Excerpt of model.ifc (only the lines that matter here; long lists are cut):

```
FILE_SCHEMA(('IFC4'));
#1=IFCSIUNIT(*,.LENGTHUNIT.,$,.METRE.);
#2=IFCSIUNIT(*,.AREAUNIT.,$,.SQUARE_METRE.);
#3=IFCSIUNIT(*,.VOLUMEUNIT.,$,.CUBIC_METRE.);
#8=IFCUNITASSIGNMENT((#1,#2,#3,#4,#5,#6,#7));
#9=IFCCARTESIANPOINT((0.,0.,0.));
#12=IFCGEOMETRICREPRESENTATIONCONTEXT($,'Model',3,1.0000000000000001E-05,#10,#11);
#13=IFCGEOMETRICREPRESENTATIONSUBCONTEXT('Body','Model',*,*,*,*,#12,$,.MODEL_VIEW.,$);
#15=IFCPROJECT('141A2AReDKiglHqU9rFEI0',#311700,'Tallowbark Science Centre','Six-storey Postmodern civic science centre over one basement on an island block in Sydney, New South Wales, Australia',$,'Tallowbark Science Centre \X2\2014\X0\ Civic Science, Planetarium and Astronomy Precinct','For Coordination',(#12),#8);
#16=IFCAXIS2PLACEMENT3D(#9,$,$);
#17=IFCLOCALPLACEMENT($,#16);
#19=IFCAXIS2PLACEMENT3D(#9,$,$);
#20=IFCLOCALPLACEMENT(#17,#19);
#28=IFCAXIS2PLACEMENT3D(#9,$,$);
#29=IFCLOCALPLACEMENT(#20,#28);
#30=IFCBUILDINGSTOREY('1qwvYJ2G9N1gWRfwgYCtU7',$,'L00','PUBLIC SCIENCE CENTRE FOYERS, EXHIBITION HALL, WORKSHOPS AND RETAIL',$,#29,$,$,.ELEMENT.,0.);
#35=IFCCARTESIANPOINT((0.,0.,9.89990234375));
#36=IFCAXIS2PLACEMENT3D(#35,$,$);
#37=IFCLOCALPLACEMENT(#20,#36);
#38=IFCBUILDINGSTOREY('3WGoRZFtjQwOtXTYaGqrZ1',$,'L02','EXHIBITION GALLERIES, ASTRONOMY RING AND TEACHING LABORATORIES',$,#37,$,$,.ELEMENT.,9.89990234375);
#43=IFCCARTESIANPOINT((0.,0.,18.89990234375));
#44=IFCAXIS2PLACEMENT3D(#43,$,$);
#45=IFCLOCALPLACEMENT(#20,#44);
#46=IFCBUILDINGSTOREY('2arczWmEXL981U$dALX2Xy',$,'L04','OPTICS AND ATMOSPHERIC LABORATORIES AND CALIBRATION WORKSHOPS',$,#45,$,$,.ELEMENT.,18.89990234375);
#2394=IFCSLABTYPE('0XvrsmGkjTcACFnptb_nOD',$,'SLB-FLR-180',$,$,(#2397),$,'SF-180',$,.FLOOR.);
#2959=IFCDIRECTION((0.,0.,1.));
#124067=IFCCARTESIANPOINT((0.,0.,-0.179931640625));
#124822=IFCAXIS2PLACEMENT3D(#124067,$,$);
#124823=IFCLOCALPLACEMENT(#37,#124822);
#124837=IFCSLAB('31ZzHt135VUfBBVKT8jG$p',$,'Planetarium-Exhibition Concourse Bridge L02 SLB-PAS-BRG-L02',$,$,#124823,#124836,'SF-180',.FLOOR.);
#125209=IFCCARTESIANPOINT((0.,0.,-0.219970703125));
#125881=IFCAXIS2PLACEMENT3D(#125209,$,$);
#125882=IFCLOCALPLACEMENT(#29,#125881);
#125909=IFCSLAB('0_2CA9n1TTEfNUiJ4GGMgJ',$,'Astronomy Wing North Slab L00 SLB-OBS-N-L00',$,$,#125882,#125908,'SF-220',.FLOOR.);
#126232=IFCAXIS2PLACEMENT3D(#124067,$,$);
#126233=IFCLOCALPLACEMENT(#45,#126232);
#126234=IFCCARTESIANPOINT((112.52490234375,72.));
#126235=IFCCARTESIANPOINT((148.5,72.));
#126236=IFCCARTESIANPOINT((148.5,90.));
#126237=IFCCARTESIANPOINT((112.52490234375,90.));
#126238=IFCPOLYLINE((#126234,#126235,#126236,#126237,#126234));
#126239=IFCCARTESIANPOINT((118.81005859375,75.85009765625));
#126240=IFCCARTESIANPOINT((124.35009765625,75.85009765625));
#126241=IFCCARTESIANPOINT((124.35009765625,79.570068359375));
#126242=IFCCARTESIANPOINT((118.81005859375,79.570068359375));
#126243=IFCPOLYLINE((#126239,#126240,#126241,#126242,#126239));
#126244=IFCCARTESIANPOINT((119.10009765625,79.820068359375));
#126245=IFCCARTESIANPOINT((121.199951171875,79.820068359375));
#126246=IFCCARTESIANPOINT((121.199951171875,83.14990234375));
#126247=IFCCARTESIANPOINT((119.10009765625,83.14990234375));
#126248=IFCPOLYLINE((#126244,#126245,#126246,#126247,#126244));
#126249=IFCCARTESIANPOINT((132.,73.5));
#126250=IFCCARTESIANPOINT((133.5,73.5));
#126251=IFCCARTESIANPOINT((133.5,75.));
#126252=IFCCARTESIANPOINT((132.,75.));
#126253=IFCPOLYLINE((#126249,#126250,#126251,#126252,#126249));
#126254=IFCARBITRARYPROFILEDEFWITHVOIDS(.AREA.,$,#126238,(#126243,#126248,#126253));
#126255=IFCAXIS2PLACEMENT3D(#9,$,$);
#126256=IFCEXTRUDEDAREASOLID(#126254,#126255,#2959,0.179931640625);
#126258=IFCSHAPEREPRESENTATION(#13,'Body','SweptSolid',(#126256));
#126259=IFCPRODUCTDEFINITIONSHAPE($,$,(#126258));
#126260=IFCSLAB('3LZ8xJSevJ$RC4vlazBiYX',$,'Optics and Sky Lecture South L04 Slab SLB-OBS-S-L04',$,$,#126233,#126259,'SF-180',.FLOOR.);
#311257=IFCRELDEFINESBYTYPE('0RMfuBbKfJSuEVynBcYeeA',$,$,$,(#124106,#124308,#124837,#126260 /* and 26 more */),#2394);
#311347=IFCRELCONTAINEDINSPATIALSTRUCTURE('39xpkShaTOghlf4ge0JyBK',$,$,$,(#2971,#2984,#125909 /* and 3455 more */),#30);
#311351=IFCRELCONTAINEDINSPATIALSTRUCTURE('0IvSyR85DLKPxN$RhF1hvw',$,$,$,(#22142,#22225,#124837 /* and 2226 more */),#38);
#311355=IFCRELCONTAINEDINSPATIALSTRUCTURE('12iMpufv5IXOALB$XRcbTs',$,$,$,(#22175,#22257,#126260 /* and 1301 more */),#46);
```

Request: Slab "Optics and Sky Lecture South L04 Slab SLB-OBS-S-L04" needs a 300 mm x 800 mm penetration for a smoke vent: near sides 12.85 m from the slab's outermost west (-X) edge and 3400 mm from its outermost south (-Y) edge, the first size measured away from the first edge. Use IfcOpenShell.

```python
import numpy as np
import ifcopenshell
import ifcopenshell.api.feature
import ifcopenshell.api.geometry
import ifcopenshell.api.root
import ifcopenshell.geom
import ifcopenshell.util.placement
import ifcopenshell.util.representation
import ifcopenshell.util.shape
import ifcopenshell.util.unit

model = ifcopenshell.open("model.ifc")
unit_scale = ifcopenshell.util.unit.calculate_unit_scale(model)
settings = ifcopenshell.geom.settings()


def volume(element):
    """Net volume in cubic metres, openings subtracted."""
    shape = ifcopenshell.geom.create_shape(settings, element)
    return ifcopenshell.util.shape.get_volume(shape.geometry)


slab = model.by_id(126260)
before = volume(slab)

# Extent in the slab's own axes, in metres. The edges named are its -X and -Y sides.
slab_shape = ifcopenshell.geom.create_shape(settings, slab)
vertices = ifcopenshell.util.shape.get_vertices(slab_shape.geometry)
x_min, y_min, bottom = vertices.min(axis=0)
top = vertices[:, 2].max()

opening = ifcopenshell.api.root.create_entity(model, ifc_class="IfcOpeningElement", name="Smoke vent opening", predefined_type="OPENING")
context = ifcopenshell.util.representation.get_context(model, "Model", "Body", "MODEL_VIEW")
width, depth = 0.3, 0.8
outline = [(0.0, 0.0), (width, 0.0), (width, depth), (0.0, depth), (0.0, 0.0)]
# Overshoot both faces by 50 mm so the cut is clean.
shape = ifcopenshell.api.geometry.add_slab_representation(
    model, context=context, depth=top - bottom + 0.1, polyline=outline
)
ifcopenshell.api.geometry.assign_representation(model, product=opening, representation=shape)

matrix = ifcopenshell.util.placement.get_local_placement(slab.ObjectPlacement)
matrix[:, 3] = matrix @ np.append(np.array([x_min + 12.85, y_min + 3.4, bottom - 0.05]) / unit_scale, 1.0)
ifcopenshell.api.geometry.edit_object_placement(model, product=opening, matrix=matrix, is_si=False)
ifcopenshell.api.feature.add_feature(model, feature=opening, element=slab)

after = volume(slab)

print(f"slab volume {before:.3f} -> {after:.3f} m3")

model.write("model_v2.ifc")
```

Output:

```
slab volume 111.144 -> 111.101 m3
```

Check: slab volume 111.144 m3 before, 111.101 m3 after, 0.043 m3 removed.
